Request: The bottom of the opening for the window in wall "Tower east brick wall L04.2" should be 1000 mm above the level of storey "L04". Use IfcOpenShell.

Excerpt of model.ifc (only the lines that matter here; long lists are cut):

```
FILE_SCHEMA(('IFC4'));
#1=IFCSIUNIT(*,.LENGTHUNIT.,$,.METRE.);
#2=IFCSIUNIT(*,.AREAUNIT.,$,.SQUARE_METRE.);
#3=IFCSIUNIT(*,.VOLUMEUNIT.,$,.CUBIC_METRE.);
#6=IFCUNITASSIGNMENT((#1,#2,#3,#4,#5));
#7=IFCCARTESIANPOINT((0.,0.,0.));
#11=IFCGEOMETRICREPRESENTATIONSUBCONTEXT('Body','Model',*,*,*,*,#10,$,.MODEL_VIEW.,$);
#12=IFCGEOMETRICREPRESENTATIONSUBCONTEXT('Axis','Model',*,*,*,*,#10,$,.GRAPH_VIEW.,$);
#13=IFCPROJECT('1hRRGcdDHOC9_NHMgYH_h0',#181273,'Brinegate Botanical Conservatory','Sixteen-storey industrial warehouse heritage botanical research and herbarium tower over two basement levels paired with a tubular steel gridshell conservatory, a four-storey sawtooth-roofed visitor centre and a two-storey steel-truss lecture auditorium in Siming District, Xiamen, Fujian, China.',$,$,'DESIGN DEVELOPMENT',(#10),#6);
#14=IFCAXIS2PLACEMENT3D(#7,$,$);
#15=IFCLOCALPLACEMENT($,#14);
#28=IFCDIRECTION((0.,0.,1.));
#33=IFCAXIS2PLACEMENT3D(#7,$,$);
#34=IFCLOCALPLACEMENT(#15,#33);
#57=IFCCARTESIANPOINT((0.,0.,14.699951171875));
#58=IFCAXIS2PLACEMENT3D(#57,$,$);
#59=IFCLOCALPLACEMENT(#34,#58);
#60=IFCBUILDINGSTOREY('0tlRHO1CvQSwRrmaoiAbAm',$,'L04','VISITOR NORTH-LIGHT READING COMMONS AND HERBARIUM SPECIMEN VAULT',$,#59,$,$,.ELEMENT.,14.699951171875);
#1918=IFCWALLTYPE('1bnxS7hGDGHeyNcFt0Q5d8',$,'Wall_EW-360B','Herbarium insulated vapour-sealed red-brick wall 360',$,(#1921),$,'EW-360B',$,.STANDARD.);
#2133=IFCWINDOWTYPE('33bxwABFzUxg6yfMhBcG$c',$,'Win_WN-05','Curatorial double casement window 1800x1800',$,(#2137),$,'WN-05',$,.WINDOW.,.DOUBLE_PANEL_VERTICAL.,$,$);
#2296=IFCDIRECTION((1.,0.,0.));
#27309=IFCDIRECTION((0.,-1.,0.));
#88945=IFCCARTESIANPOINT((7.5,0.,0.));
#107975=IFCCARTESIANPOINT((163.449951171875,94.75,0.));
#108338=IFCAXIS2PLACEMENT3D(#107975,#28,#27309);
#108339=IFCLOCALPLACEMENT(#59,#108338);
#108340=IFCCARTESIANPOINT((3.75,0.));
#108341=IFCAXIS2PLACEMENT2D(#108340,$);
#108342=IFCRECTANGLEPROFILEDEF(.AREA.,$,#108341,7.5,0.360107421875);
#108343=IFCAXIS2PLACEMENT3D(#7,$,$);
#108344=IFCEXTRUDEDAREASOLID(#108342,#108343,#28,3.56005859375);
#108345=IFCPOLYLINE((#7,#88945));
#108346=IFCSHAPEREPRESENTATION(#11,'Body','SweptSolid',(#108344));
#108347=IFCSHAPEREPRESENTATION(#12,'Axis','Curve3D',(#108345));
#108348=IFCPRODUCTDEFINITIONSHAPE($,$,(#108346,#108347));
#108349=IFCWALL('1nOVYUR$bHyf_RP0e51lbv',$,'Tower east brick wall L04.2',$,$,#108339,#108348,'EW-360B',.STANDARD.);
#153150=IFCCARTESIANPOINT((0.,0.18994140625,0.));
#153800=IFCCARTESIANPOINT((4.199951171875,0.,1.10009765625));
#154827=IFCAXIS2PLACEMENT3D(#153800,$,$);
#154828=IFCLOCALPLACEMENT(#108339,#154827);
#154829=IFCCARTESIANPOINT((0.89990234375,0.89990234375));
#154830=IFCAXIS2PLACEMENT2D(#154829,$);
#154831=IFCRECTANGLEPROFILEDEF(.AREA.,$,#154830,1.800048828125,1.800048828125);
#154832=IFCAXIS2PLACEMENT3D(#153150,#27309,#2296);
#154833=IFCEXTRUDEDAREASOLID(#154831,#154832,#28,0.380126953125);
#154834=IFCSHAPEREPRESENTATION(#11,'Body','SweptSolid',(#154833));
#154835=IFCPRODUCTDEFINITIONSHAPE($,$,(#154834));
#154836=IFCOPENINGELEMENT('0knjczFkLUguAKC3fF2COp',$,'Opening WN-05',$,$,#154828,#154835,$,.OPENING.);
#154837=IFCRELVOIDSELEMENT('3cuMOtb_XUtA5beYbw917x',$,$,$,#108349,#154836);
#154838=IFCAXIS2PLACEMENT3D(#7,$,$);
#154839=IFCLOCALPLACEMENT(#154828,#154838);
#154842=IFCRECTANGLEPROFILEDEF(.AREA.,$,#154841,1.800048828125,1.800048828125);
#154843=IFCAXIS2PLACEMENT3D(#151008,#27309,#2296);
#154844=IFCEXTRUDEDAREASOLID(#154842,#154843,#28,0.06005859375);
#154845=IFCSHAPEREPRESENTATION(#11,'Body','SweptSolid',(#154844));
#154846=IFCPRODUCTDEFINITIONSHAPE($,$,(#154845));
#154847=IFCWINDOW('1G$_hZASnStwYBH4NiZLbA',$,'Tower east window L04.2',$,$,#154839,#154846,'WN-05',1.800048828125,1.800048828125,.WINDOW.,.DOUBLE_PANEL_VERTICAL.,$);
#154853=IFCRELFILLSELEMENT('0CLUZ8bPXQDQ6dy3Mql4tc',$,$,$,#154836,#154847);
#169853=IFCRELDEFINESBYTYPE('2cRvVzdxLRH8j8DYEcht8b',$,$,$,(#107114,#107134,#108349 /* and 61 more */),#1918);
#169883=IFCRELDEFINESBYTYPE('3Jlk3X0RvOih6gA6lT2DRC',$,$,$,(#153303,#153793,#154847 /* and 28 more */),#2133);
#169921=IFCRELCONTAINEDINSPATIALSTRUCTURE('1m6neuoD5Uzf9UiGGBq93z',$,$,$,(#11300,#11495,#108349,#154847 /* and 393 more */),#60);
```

```python
import numpy as np
import ifcopenshell
import ifcopenshell.api.geometry
import ifcopenshell.geom
import ifcopenshell.util.element
import ifcopenshell.util.placement
import ifcopenshell.util.shape
import ifcopenshell.util.unit

model = ifcopenshell.open("model.ifc")
unit_scale = ifcopenshell.util.unit.calculate_unit_scale(model)

window = model.by_id(154847)
opening = window.FillsVoids[0].RelatingOpeningElement
storey = ifcopenshell.util.element.get_container(window, ifc_class="IfcBuildingStorey")
level = ifcopenshell.util.placement.get_local_placement(storey.ObjectPlacement)[2, 3]

# The opening's origin need not be at the sill, so measure its lowest point.
shape = ifcopenshell.geom.create_shape(ifcopenshell.geom.settings(), opening)
bottom = ifcopenshell.util.shape.get_shape_bottom_elevation(shape, shape.geometry) / unit_scale
dz = level + 1.0 - bottom

shift = np.array([0.0, 0.0, dz])
# The window is placed relative to its opening, so it follows when the opening moves.
matrix = ifcopenshell.util.placement.get_local_placement(opening.ObjectPlacement)
matrix[:3, 3] += shift
ifcopenshell.api.geometry.edit_object_placement(
    model, product=opening, matrix=matrix, is_si=False, should_transform_children=True
)

print(f"moved by {dz * unit_scale:+.3f} m")

model.write("model_rev.ifc")
```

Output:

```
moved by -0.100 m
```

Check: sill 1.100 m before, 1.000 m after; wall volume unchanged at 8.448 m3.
